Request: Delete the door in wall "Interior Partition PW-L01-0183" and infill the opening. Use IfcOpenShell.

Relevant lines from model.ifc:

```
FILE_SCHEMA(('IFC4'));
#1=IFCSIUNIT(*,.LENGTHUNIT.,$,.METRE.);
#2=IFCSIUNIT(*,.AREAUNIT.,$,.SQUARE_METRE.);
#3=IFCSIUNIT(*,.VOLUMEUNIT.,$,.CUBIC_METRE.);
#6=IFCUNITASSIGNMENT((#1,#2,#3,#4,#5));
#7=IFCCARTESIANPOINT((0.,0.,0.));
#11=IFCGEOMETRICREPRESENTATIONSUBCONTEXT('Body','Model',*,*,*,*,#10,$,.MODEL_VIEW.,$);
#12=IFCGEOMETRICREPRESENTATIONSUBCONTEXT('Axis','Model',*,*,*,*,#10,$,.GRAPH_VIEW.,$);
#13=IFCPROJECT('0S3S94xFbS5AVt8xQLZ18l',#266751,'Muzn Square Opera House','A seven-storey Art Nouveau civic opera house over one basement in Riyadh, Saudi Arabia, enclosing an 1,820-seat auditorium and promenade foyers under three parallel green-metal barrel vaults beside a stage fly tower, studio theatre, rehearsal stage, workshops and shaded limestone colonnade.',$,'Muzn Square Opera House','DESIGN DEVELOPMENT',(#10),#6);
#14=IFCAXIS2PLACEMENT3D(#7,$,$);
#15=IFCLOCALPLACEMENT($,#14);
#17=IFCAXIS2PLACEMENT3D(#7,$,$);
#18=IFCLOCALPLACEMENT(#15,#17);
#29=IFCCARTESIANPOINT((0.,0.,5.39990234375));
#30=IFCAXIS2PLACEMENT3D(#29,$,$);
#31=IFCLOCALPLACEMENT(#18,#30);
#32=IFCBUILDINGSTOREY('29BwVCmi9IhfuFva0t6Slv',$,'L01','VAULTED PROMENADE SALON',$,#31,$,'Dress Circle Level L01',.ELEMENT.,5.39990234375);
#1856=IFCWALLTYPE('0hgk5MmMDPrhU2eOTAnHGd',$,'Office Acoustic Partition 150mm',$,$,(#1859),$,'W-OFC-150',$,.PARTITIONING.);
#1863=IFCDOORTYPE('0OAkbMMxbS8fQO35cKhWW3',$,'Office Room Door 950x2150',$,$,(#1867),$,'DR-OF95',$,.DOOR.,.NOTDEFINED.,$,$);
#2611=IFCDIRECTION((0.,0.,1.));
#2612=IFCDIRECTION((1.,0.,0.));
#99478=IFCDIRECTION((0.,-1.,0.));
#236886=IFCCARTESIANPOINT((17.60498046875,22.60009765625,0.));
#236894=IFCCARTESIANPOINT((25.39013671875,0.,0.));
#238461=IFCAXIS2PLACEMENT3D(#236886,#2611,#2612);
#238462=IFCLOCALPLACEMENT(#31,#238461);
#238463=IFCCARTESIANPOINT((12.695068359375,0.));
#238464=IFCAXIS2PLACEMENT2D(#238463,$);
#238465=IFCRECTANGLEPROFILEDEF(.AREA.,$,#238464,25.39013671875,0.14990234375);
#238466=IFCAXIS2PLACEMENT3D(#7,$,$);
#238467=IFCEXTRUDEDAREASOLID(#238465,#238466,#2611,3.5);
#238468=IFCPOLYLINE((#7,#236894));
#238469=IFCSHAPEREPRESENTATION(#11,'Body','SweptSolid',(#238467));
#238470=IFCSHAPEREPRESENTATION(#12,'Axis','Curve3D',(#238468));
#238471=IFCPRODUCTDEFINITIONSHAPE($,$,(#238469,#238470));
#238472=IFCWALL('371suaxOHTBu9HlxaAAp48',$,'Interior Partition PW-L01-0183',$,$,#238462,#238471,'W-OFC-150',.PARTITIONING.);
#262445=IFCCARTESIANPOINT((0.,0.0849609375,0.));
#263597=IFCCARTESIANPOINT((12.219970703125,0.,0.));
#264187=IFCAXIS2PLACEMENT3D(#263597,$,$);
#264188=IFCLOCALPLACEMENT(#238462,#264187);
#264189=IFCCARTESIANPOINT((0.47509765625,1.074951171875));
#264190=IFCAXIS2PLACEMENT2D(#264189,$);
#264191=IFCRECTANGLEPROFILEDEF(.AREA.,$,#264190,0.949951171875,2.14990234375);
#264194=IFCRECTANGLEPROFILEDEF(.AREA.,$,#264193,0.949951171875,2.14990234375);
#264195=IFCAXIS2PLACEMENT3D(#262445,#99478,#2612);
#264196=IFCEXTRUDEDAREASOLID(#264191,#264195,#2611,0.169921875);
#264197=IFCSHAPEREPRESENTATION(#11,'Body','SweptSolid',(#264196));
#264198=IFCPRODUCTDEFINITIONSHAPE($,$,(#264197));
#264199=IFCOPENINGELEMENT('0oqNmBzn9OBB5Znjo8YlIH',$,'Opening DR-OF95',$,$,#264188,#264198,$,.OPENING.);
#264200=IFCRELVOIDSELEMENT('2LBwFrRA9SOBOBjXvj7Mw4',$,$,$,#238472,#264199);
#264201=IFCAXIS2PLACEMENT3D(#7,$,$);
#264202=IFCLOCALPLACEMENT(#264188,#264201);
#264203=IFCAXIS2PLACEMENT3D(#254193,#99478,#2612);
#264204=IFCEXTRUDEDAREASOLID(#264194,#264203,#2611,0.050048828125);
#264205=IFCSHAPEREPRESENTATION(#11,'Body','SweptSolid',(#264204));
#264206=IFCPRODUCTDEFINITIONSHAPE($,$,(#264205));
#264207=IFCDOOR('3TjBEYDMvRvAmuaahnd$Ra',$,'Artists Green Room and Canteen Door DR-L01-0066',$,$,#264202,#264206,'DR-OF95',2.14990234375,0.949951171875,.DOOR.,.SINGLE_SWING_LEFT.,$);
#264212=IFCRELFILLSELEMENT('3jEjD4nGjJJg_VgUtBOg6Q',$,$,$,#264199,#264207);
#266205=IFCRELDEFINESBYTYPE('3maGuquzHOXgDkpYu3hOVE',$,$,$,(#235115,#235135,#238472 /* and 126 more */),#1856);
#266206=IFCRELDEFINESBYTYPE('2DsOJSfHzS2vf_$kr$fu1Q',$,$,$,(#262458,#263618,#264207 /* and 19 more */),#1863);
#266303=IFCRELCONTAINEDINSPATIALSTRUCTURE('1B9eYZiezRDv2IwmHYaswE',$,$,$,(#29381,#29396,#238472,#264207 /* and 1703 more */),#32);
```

```python
import ifcopenshell
import ifcopenshell.api.feature
import ifcopenshell.api.root
import ifcopenshell.geom
import ifcopenshell.util.shape

model = ifcopenshell.open("model.ifc")
settings = ifcopenshell.geom.settings()


def volume(element):
    """Net volume in cubic metres, openings subtracted."""
    shape = ifcopenshell.geom.create_shape(settings, element)
    return ifcopenshell.util.shape.get_volume(shape.geometry)


door = model.by_guid("3TjBEYDMvRvAmuaahnd$Ra")
opening = door.FillsVoids[0].RelatingOpeningElement
wall = opening.VoidsElements[0].RelatingBuildingElement
before = volume(wall)

ifcopenshell.api.root.remove_product(model, product=door)
ifcopenshell.api.feature.remove_feature(model, feature=opening)

after = volume(wall)

print(f"wall volume {before:.3f} -> {after:.3f} m3")

model.write("model_v2.ifc")
```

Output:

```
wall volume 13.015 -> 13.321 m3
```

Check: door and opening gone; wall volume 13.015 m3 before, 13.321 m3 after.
